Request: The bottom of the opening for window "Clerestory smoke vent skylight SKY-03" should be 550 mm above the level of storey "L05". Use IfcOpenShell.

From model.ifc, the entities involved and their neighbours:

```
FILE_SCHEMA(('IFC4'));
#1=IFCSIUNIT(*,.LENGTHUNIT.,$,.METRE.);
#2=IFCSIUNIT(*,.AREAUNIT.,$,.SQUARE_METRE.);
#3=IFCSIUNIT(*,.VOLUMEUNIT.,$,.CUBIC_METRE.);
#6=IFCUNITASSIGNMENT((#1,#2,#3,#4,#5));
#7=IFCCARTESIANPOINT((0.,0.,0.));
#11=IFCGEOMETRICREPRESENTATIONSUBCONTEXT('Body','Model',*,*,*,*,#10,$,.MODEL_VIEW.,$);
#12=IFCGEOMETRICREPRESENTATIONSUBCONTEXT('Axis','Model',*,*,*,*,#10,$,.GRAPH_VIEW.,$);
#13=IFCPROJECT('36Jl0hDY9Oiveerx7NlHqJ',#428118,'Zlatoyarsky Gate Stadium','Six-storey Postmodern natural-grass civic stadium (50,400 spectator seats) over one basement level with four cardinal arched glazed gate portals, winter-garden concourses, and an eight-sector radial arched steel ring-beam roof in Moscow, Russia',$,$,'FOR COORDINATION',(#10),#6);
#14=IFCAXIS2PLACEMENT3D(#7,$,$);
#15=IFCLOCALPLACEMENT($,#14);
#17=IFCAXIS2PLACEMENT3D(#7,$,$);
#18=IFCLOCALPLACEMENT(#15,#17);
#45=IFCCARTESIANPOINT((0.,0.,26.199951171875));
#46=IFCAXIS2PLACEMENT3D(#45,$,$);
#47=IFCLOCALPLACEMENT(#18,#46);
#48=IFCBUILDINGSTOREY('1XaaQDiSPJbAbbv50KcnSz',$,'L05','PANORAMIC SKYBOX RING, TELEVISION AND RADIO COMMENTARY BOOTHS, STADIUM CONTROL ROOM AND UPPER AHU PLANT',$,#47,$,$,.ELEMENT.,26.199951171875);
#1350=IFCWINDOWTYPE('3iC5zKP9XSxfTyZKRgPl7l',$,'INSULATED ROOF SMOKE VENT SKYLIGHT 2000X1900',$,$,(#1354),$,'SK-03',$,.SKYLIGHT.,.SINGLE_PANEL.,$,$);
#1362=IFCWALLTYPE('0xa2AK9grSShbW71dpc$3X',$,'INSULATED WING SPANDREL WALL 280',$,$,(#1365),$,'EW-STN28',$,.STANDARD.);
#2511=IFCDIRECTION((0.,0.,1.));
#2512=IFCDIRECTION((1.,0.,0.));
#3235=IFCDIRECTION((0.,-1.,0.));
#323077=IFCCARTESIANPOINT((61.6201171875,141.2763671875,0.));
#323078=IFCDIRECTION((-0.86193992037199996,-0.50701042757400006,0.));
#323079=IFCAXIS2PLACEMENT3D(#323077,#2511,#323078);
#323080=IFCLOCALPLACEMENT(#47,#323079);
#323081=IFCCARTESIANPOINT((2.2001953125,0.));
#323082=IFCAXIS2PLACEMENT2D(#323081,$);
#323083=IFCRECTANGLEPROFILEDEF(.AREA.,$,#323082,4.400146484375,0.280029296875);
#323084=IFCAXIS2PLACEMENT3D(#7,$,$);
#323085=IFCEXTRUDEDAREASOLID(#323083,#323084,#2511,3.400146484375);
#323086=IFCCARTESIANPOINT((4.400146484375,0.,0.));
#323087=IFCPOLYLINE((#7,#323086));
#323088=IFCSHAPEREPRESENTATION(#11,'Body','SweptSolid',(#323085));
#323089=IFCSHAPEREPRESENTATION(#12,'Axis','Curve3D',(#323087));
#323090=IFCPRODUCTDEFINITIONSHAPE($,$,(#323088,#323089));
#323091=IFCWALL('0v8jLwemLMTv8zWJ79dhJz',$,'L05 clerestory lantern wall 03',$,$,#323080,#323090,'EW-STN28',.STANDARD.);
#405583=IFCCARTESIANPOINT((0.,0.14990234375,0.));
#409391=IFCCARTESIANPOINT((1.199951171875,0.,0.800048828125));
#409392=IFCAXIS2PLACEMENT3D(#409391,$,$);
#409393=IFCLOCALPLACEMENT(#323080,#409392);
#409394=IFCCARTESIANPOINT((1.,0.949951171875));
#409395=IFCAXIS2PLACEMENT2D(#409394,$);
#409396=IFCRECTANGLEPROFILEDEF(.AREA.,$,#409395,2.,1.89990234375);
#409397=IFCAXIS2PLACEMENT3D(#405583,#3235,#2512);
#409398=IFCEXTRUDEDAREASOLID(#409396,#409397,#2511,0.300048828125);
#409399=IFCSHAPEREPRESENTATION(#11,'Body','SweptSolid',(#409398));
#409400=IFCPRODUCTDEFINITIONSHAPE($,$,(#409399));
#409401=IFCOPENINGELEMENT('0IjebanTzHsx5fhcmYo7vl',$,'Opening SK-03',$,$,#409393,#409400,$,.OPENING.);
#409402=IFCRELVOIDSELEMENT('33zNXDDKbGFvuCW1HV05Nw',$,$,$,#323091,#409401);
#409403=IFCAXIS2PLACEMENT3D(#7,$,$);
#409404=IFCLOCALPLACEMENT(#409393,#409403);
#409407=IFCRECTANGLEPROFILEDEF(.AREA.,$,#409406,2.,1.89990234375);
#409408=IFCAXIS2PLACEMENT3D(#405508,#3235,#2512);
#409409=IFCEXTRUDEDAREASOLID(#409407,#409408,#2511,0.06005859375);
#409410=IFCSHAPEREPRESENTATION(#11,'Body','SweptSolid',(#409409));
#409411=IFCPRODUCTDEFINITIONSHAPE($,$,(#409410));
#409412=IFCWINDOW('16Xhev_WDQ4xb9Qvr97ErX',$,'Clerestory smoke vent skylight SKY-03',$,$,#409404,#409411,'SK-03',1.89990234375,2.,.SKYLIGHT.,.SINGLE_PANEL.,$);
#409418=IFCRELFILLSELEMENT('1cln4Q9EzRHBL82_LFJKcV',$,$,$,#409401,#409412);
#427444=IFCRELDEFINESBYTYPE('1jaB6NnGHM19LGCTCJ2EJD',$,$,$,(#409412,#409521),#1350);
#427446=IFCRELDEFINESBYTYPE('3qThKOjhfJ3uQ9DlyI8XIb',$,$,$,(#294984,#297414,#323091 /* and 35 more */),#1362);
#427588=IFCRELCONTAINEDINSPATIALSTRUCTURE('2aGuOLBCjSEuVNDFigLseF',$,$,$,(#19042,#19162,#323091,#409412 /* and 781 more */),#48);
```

```python
import numpy as np
import ifcopenshell
import ifcopenshell.api.geometry
import ifcopenshell.geom
import ifcopenshell.util.element
import ifcopenshell.util.placement
import ifcopenshell.util.shape
import ifcopenshell.util.unit

model = ifcopenshell.open("model.ifc")
unit_scale = ifcopenshell.util.unit.calculate_unit_scale(model)

window = model.by_id(409412)
opening = window.FillsVoids[0].RelatingOpeningElement
storey = ifcopenshell.util.element.get_container(window, ifc_class="IfcBuildingStorey")
level = ifcopenshell.util.placement.get_local_placement(storey.ObjectPlacement)[2, 3]

# The opening's origin need not be at the sill, so measure its lowest point.
shape = ifcopenshell.geom.create_shape(ifcopenshell.geom.settings(), opening)
bottom = ifcopenshell.util.shape.get_shape_bottom_elevation(shape, shape.geometry) / unit_scale
dz = level + 0.55 - bottom

shift = np.array([0.0, 0.0, dz])
# The window is placed relative to its opening, so it follows when the opening moves.
matrix = ifcopenshell.util.placement.get_local_placement(opening.ObjectPlacement)
matrix[:3, 3] += shift
ifcopenshell.api.geometry.edit_object_placement(
    model, product=opening, matrix=matrix, is_si=False, should_transform_children=True
)

print(f"moved by {dz * unit_scale:+.3f} m")

model.write("model_rev.ifc")
```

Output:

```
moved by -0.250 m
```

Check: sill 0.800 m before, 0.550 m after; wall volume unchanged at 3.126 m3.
